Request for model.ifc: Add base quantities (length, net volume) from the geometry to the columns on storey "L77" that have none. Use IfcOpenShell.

First a look at what the model holds.

```python
import ifcopenshell
import ifcopenshell.util.element
import ifcopenshell.util.unit

model = ifcopenshell.open("model.ifc")
print(model.schema)
for unit_type in ("LENGTHUNIT", "AREAUNIT", "VOLUMEUNIT"):
    print(unit_type, ifcopenshell.util.unit.calculate_unit_scale(model, unit_type))
storey = next(s for s in model.by_type("IfcBuildingStorey") if s.Name == "L77")
columns = [e for e in ifcopenshell.util.element.get_decomposition(storey) if e.is_a("IfcColumn")]
for e in sorted(columns, key=lambda e: e.id()):
    print(e.id(), e.is_a(), e.Name, list(ifcopenshell.util.element.get_psets(e, qtos_only=True)), sep=" | ")
```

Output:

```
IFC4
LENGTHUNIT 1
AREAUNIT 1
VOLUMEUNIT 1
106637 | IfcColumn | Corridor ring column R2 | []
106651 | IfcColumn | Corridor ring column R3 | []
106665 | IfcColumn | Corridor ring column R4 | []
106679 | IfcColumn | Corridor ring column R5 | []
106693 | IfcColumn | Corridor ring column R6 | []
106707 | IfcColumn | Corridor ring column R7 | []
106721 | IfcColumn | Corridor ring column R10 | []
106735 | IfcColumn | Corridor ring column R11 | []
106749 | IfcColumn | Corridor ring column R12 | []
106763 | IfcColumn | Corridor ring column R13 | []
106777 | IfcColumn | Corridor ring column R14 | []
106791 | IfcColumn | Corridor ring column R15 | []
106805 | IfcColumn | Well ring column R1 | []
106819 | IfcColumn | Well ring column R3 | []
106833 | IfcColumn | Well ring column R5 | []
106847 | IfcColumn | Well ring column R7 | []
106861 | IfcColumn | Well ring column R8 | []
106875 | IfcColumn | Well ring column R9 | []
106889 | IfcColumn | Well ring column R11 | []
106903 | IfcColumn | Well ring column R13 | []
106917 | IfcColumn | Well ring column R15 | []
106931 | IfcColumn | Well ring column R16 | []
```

```python
import ifcopenshell
import ifcopenshell.api.pset
import ifcopenshell.geom
import ifcopenshell.util.element
import ifcopenshell.util.shape
import ifcopenshell.util.unit

model = ifcopenshell.open("model.ifc")
unit_scale = ifcopenshell.util.unit.calculate_unit_scale(model)
volume_scale = ifcopenshell.util.unit.calculate_unit_scale(model, "VOLUMEUNIT")
settings = ifcopenshell.geom.settings()

storey = next(s for s in model.by_type("IfcBuildingStorey") if s.Name == "L77")
columns = [e for e in ifcopenshell.util.element.get_decomposition(storey) if e.is_a("IfcColumn")]

for e in sorted(columns, key=lambda e: e.id()):
    if ifcopenshell.util.element.get_psets(e, qtos_only=True, should_inherit=False):
        continue
    # Geometry comes back in metres, in the element's own axes.
    shape = ifcopenshell.geom.create_shape(settings, e)
    values = {
        "Length": ifcopenshell.util.shape.get_z(shape.geometry) / unit_scale,
        "NetVolume": ifcopenshell.util.shape.get_volume(shape.geometry) / volume_scale,
    }
    qto = ifcopenshell.api.pset.add_qto(model, product=e, name="Qto_ColumnBaseQuantities")
    ifcopenshell.api.pset.edit_qto(model, qto=qto, properties=values)
    print(e.id(), {k: round(v, 3) for k, v in values.items()})

model.write("model_updated.ifc")
```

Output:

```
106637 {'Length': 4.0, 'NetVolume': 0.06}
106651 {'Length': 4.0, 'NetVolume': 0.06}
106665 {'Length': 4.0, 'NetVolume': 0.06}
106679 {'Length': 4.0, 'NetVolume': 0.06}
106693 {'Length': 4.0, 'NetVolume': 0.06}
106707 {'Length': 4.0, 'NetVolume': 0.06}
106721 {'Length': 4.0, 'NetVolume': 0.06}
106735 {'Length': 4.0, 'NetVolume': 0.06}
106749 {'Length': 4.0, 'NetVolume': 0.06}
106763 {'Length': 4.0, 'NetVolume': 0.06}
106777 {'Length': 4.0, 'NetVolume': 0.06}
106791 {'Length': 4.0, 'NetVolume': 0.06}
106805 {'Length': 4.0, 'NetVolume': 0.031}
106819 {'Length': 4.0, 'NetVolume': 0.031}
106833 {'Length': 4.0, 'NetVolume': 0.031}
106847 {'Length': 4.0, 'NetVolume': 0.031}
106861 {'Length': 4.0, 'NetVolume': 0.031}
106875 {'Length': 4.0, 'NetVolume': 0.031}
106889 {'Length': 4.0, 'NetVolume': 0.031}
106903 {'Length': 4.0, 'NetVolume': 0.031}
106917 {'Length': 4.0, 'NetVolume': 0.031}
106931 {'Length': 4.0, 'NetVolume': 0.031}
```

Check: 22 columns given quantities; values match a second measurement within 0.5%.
